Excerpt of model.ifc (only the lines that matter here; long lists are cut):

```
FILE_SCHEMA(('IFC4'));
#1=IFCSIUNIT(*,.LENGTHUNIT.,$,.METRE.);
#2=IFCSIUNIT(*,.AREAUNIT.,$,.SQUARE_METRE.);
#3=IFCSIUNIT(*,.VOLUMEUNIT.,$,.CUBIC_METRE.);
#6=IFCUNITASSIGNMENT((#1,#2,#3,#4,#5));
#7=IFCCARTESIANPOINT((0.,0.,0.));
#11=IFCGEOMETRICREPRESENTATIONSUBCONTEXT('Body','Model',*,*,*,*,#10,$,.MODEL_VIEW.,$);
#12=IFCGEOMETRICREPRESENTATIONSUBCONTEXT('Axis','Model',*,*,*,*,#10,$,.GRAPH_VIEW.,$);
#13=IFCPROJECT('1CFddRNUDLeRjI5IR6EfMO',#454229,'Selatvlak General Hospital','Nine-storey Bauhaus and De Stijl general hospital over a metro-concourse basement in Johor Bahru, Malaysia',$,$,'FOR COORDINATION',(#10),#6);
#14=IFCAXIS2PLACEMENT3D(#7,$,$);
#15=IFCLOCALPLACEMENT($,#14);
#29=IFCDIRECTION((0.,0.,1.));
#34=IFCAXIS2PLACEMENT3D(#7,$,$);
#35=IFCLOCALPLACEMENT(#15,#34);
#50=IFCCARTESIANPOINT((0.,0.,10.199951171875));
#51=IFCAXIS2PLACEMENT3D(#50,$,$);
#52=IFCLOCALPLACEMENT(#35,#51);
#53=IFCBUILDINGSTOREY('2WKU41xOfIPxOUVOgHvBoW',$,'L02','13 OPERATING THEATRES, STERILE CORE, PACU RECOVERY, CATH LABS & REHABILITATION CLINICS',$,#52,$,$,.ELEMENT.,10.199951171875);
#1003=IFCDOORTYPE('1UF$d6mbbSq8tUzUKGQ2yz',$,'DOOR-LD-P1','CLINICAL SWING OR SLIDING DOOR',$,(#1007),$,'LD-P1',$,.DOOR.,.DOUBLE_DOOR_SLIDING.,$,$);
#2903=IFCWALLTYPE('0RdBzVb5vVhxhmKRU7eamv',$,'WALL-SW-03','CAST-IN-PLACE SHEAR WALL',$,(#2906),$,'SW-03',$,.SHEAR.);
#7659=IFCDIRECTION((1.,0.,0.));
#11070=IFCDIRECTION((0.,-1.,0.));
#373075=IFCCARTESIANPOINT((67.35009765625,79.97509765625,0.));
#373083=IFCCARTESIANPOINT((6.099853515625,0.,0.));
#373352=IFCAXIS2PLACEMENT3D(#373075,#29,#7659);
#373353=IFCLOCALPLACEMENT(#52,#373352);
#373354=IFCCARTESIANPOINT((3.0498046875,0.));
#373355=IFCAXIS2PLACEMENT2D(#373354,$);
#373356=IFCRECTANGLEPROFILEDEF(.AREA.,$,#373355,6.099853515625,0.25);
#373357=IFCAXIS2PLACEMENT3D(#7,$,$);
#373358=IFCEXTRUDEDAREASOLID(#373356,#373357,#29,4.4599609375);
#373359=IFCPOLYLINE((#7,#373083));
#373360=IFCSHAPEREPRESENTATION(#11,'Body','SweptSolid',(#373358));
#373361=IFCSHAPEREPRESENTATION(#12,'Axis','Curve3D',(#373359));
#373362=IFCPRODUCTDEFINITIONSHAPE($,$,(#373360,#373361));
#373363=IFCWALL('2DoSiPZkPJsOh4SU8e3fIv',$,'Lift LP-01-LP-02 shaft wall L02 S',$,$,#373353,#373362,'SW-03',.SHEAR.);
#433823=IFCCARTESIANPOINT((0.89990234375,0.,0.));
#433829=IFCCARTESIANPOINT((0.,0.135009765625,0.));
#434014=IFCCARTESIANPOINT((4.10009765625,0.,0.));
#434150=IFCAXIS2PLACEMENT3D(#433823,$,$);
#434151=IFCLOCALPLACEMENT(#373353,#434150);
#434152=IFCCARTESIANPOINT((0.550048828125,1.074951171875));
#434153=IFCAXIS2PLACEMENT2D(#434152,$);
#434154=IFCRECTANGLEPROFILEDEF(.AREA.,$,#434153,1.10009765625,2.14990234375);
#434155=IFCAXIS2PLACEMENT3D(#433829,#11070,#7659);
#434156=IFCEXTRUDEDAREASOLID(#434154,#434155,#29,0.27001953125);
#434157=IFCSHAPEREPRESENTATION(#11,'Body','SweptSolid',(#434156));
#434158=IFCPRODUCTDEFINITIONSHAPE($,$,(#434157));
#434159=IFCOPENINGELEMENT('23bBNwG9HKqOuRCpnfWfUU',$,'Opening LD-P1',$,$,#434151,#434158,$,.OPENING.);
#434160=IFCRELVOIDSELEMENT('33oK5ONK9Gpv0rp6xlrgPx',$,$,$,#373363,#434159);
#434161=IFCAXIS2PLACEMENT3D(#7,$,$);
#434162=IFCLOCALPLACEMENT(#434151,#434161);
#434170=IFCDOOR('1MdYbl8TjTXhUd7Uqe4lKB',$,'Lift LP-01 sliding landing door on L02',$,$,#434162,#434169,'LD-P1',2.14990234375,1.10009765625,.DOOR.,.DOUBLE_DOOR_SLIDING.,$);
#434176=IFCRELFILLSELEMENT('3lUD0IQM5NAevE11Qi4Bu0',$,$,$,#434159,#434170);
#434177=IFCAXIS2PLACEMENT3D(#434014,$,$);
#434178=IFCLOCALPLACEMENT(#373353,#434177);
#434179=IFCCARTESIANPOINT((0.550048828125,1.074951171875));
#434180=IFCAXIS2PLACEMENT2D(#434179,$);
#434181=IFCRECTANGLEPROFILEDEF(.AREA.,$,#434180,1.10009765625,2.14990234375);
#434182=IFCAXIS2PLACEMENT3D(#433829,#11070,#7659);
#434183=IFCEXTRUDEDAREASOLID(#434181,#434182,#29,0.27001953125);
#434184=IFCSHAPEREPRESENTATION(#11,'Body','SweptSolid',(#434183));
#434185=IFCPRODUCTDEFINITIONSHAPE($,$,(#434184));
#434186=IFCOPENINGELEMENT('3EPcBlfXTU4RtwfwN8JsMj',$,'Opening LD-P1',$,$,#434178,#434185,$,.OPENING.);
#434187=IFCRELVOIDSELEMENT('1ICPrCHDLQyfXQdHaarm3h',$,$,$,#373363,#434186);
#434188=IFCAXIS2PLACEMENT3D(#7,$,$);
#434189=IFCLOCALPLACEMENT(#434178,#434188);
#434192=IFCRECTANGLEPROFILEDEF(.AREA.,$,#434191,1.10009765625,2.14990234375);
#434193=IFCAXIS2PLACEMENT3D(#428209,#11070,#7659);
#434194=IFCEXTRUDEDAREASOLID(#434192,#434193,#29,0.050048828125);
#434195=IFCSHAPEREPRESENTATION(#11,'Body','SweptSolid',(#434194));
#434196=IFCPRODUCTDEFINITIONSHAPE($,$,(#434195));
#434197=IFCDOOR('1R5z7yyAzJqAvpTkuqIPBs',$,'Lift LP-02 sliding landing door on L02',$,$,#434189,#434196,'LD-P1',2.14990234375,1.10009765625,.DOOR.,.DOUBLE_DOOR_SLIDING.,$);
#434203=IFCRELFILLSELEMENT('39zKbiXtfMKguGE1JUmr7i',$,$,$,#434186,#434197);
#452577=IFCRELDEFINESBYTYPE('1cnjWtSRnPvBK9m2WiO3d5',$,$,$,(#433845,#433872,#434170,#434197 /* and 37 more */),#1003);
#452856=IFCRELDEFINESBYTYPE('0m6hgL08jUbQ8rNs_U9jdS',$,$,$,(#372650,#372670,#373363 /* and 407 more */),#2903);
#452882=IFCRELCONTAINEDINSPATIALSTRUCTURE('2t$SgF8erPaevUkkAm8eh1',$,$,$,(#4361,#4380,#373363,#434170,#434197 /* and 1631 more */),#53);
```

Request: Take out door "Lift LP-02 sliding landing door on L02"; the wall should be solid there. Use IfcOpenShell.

```python
import ifcopenshell
import ifcopenshell.api.feature
import ifcopenshell.api.root
import ifcopenshell.geom
import ifcopenshell.util.shape

model = ifcopenshell.open("model.ifc")
settings = ifcopenshell.geom.settings()


def volume(element):
    """Net volume in cubic metres, openings subtracted."""
    shape = ifcopenshell.geom.create_shape(settings, element)
    return ifcopenshell.util.shape.get_volume(shape.geometry)


door = model.by_id(434197)
opening = door.FillsVoids[0].RelatingOpeningElement
wall = opening.VoidsElements[0].RelatingBuildingElement
before = volume(wall)

ifcopenshell.api.root.remove_product(model, product=door)
ifcopenshell.api.feature.remove_feature(model, feature=opening)

after = volume(wall)

print(f"wall volume {before:.3f} -> {after:.3f} m3")

model.write("model-out.ifc")
```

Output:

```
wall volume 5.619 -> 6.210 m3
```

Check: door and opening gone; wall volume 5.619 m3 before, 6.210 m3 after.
